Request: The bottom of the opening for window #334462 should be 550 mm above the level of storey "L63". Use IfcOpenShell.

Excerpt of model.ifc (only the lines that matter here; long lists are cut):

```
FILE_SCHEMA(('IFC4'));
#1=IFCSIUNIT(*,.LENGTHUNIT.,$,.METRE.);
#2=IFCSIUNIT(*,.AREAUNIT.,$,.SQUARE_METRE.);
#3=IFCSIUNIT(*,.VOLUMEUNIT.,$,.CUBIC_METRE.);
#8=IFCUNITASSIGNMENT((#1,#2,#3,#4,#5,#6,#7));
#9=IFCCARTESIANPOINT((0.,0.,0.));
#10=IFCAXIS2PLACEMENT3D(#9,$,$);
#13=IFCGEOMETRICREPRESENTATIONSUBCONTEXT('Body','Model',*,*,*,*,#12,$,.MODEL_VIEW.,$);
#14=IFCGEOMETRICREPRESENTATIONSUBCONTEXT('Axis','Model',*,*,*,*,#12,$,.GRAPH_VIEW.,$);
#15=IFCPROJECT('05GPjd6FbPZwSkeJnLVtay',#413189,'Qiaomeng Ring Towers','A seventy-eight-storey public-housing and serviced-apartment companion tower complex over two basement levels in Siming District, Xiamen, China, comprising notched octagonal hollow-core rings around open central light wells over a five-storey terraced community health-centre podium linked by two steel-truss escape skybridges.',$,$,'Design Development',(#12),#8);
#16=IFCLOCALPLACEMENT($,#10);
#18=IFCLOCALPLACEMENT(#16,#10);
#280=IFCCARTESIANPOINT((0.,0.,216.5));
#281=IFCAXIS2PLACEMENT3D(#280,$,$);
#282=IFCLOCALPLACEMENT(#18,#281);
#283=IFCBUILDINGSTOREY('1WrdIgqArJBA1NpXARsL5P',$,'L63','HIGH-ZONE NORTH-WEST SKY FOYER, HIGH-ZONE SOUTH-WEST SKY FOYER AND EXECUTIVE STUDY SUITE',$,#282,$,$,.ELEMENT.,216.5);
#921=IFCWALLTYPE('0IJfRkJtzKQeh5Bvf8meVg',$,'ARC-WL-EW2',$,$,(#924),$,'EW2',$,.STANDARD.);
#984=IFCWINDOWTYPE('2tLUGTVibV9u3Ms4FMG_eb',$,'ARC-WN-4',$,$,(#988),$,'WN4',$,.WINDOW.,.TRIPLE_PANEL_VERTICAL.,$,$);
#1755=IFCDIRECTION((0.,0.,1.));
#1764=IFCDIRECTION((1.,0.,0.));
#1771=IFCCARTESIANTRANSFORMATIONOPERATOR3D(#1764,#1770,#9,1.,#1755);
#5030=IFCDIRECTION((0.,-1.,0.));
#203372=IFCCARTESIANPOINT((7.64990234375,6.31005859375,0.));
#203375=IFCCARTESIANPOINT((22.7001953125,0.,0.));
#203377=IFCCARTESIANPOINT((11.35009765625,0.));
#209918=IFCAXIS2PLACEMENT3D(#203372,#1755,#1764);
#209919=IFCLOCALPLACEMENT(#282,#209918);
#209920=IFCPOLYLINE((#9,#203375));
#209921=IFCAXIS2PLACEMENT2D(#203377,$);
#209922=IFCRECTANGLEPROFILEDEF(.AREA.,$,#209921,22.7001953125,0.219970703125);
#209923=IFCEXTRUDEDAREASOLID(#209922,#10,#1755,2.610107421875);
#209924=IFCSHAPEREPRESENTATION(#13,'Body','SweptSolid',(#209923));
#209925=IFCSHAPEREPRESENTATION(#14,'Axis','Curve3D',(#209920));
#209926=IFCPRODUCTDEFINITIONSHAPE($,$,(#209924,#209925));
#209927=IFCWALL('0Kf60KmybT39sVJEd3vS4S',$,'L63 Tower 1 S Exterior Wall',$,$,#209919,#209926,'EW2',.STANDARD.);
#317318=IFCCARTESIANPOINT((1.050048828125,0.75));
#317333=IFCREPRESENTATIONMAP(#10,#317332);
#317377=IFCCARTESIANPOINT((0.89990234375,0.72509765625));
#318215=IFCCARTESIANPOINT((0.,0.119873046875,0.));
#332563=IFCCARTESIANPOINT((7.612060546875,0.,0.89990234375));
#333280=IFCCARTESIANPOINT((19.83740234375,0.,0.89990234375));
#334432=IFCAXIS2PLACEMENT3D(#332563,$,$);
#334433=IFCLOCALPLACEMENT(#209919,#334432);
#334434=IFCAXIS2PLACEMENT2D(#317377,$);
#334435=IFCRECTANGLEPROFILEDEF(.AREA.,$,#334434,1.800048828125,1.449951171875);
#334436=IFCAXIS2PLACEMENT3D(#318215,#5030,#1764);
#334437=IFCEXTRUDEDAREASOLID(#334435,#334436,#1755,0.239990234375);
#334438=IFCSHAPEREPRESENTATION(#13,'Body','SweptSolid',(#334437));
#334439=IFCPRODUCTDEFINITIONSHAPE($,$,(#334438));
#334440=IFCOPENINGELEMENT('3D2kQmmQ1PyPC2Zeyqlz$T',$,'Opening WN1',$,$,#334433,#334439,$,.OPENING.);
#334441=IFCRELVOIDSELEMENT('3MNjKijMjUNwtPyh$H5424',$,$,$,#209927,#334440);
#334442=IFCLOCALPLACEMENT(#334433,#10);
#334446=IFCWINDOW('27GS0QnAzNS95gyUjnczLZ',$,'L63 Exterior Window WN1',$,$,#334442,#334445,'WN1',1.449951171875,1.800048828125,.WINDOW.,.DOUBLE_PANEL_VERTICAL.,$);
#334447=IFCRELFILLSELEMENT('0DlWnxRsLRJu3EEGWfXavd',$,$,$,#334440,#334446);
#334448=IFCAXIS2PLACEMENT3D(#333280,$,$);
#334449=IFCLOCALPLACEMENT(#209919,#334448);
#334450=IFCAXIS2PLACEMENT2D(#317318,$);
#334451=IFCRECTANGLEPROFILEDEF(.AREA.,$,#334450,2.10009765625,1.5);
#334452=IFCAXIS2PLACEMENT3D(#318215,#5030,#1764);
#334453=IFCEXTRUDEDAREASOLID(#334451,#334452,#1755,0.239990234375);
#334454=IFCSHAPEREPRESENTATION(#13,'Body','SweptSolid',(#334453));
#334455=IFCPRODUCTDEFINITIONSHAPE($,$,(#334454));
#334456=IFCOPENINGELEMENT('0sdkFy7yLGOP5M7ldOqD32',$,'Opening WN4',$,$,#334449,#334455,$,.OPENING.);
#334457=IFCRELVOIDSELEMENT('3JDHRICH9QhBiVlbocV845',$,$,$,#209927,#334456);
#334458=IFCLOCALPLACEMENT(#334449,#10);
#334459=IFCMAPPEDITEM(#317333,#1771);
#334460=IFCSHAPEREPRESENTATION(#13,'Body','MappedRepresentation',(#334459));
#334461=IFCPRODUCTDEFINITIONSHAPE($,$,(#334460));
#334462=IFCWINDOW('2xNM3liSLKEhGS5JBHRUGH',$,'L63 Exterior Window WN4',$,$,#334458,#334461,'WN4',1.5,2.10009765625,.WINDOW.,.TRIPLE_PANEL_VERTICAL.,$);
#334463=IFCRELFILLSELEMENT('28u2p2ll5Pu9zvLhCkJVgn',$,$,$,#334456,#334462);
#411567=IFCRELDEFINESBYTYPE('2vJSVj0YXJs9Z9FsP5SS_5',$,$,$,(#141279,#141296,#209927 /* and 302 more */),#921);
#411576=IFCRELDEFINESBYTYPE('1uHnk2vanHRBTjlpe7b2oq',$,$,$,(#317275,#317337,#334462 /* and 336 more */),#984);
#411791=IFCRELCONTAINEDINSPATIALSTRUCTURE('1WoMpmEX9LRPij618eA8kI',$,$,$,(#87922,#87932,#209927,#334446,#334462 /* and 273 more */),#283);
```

```python
import numpy as np
import ifcopenshell
import ifcopenshell.api.geometry
import ifcopenshell.geom
import ifcopenshell.util.element
import ifcopenshell.util.placement
import ifcopenshell.util.shape
import ifcopenshell.util.unit

model = ifcopenshell.open("model.ifc")
unit_scale = ifcopenshell.util.unit.calculate_unit_scale(model)

window = model.by_guid("2xNM3liSLKEhGS5JBHRUGH")
opening = window.FillsVoids[0].RelatingOpeningElement
storey = ifcopenshell.util.element.get_container(window, ifc_class="IfcBuildingStorey")
level = ifcopenshell.util.placement.get_local_placement(storey.ObjectPlacement)[2, 3]

# The opening's origin need not be at the sill, so measure its lowest point.
shape = ifcopenshell.geom.create_shape(ifcopenshell.geom.settings(), opening)
bottom = ifcopenshell.util.shape.get_shape_bottom_elevation(shape, shape.geometry) / unit_scale
dz = level + 0.55 - bottom

shift = np.array([0.0, 0.0, dz])
# The window is placed relative to its opening, so it follows when the opening moves.
matrix = ifcopenshell.util.placement.get_local_placement(opening.ObjectPlacement)
matrix[:3, 3] += shift
ifcopenshell.api.geometry.edit_object_placement(
    model, product=opening, matrix=matrix, is_si=False, should_transform_children=True
)

print(f"moved by {dz * unit_scale:+.3f} m")

model.write("model_rev.ifc")
```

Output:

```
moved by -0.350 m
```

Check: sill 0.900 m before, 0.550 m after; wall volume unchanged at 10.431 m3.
